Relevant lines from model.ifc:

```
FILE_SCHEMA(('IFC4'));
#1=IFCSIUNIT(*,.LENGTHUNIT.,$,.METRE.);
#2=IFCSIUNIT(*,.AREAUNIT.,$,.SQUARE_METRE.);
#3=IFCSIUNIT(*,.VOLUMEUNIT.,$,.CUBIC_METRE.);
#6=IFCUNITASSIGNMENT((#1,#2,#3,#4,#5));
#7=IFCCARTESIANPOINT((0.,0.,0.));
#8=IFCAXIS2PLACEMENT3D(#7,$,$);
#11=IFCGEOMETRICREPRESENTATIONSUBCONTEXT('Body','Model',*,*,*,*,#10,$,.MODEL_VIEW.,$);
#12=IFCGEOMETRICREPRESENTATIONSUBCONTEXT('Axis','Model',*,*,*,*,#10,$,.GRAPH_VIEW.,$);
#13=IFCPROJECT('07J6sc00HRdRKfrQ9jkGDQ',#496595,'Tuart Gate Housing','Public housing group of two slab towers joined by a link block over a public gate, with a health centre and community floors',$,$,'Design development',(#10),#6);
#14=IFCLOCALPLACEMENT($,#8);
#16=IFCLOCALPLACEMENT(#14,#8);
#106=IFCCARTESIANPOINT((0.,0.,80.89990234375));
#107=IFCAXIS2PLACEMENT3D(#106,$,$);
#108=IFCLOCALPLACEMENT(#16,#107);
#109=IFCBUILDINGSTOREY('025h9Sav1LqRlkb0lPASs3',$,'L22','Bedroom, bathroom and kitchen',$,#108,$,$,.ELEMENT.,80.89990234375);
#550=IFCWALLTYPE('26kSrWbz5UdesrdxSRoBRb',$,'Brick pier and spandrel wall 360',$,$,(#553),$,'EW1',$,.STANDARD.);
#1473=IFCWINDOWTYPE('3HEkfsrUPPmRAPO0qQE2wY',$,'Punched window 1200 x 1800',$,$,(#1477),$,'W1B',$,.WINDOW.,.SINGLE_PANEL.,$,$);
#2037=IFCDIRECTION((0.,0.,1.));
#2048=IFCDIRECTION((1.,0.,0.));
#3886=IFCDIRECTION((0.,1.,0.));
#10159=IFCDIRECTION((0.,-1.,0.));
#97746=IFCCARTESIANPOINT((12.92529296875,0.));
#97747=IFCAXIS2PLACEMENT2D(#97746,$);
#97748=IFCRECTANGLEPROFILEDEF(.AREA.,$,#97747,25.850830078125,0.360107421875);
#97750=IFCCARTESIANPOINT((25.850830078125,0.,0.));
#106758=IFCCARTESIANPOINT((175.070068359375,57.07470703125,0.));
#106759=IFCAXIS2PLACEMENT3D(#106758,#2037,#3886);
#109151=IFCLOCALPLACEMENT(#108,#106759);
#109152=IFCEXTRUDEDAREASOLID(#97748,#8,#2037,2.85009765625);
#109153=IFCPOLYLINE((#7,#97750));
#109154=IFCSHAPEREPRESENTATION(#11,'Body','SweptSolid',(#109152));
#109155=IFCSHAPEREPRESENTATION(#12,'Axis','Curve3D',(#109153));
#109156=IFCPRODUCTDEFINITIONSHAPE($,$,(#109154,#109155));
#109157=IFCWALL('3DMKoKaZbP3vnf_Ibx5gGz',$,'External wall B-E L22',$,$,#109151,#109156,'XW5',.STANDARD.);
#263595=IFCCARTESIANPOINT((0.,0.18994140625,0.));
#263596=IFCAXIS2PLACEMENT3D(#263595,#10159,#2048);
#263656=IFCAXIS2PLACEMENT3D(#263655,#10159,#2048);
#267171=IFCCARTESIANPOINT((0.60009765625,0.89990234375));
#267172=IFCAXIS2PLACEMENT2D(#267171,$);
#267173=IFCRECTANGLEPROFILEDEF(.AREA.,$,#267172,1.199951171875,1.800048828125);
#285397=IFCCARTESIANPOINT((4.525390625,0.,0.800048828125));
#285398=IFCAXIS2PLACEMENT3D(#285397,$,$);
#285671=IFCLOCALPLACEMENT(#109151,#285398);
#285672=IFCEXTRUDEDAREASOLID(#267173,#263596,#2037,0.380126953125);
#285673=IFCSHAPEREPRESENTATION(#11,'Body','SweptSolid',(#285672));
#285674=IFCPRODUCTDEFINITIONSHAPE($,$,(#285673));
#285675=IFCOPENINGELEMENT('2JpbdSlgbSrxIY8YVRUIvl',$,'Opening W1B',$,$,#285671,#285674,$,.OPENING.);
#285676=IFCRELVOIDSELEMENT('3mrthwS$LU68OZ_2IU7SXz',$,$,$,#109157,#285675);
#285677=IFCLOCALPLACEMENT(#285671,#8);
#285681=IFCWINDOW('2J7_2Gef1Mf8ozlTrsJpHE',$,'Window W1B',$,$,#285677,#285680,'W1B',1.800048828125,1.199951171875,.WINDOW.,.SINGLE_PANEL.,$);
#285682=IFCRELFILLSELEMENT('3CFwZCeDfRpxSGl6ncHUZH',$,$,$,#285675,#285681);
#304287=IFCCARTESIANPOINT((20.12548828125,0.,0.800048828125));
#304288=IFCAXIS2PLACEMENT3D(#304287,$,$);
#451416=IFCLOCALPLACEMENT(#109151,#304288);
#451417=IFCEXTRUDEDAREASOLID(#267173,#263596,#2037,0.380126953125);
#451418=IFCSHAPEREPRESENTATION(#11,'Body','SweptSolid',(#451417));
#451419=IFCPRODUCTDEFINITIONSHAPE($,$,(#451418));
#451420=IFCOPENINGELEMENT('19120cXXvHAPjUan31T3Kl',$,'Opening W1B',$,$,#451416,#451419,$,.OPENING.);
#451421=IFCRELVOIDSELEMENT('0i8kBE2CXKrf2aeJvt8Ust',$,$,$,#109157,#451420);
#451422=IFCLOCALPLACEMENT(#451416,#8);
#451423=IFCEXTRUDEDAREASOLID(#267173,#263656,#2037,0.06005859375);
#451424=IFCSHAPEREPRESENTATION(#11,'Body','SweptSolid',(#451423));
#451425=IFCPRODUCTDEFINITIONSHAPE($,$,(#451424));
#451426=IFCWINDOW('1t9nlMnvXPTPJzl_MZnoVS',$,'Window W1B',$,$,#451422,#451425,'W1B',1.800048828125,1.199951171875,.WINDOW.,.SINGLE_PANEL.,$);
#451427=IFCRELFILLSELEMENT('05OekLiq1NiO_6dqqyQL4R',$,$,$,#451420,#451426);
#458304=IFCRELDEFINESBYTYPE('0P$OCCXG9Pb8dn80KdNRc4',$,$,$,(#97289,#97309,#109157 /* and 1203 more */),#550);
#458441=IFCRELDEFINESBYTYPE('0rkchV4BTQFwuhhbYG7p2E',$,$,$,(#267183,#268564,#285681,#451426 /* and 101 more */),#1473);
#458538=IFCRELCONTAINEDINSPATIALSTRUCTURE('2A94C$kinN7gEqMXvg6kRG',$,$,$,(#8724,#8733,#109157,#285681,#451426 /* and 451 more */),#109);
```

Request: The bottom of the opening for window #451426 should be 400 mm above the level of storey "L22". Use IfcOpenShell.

```python
import numpy as np
import ifcopenshell
import ifcopenshell.api.geometry
import ifcopenshell.geom
import ifcopenshell.util.element
import ifcopenshell.util.placement
import ifcopenshell.util.shape
import ifcopenshell.util.unit

model = ifcopenshell.open("model.ifc")
unit_scale = ifcopenshell.util.unit.calculate_unit_scale(model)

window = model.by_guid("1t9nlMnvXPTPJzl_MZnoVS")
opening = window.FillsVoids[0].RelatingOpeningElement
storey = ifcopenshell.util.element.get_container(window, ifc_class="IfcBuildingStorey")
level = ifcopenshell.util.placement.get_local_placement(storey.ObjectPlacement)[2, 3]

# The opening's origin need not be at the sill, so measure its lowest point.
shape = ifcopenshell.geom.create_shape(ifcopenshell.geom.settings(), opening)
bottom = ifcopenshell.util.shape.get_shape_bottom_elevation(shape, shape.geometry) / unit_scale
dz = level + 0.4 / unit_scale - bottom

shift = np.array([0.0, 0.0, dz])
# The window is placed relative to its opening, so it follows when the opening moves.
matrix = ifcopenshell.util.placement.get_local_placement(opening.ObjectPlacement)
matrix[:3, 3] += shift
ifcopenshell.api.geometry.edit_object_placement(
    model, product=opening, matrix=matrix, is_si=False, should_transform_children=True
)

print(f"moved by {dz * unit_scale:+.3f} m")

model.write("model_updated.ifc")
```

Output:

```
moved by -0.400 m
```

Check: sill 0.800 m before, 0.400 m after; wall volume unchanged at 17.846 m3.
